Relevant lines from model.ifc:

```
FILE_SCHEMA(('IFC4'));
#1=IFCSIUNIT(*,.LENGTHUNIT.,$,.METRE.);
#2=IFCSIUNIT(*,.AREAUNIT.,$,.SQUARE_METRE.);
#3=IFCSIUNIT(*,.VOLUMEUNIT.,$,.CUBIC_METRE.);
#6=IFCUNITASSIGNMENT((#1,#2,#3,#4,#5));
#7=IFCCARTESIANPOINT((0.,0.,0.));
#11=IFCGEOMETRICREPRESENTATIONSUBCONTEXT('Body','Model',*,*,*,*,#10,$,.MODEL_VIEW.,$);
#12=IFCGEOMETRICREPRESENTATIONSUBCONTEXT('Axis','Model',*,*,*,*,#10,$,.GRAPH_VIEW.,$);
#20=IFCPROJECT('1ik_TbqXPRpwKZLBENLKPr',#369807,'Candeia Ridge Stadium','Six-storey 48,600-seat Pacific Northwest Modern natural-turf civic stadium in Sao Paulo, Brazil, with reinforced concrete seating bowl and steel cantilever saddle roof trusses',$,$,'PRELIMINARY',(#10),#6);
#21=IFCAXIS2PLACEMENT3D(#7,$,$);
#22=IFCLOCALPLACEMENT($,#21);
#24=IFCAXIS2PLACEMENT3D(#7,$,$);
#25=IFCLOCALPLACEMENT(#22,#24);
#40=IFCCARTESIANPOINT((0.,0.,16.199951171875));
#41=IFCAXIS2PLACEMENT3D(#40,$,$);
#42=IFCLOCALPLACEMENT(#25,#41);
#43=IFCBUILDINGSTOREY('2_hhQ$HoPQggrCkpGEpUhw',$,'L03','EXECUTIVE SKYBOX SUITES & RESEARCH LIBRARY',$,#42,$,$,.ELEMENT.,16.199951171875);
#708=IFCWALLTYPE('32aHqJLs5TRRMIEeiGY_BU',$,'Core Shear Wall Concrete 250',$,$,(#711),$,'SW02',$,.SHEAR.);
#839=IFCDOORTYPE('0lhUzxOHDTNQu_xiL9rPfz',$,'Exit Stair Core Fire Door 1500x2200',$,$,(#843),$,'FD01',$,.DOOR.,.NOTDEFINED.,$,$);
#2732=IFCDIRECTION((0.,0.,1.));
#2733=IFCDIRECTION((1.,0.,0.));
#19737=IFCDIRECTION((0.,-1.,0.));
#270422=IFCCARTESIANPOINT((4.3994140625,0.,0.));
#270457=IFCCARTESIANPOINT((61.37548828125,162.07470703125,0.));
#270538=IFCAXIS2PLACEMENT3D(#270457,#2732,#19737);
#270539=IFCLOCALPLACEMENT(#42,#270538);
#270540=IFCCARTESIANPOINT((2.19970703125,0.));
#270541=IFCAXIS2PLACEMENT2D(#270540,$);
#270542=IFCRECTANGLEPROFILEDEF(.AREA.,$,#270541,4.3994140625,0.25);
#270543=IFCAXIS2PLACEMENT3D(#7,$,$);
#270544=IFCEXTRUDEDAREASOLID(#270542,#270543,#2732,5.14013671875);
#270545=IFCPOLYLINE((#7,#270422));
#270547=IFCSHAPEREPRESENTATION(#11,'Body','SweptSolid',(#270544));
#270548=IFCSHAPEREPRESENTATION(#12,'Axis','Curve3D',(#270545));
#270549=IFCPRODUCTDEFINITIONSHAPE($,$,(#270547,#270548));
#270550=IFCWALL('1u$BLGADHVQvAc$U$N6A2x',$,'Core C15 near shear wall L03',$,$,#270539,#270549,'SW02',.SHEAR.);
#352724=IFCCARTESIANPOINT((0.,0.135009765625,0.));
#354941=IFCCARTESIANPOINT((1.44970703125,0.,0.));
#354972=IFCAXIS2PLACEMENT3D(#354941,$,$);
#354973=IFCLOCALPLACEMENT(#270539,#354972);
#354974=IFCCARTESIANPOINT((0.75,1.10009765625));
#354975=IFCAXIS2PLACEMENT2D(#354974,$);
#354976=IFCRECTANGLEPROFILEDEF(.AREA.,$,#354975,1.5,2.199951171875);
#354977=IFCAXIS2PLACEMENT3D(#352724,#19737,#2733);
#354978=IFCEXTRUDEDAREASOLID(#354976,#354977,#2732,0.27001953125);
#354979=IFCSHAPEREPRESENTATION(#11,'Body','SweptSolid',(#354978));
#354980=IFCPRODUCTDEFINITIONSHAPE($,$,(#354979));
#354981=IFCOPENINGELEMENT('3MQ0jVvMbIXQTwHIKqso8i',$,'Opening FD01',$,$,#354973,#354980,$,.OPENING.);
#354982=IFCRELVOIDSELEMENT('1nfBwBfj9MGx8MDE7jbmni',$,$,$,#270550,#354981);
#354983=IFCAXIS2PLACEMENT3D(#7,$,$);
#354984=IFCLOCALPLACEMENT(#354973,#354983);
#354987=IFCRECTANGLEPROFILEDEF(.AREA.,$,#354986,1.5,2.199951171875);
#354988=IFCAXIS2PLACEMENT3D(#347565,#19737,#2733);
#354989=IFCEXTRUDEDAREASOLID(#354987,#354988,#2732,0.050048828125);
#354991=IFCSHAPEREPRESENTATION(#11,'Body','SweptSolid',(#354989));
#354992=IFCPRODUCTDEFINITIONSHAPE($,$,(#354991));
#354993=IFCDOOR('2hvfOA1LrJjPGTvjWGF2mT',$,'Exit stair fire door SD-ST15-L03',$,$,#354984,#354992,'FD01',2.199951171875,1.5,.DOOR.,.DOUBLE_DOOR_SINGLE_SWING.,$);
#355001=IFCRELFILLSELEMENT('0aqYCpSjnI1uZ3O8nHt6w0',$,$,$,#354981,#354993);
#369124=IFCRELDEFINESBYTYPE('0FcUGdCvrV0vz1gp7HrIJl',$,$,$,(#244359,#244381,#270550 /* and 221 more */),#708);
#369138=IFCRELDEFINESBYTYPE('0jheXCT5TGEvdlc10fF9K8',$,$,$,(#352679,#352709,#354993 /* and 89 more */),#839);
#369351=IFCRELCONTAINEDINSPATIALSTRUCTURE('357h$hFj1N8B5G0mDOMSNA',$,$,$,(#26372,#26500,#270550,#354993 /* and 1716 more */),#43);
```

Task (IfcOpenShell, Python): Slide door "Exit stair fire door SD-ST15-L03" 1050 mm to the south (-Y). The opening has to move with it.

```python
import ifcopenshell
import ifcopenshell.api.geometry
import ifcopenshell.util.placement
import ifcopenshell.util.unit

model = ifcopenshell.open("model.ifc")
unit_scale = ifcopenshell.util.unit.calculate_unit_scale(model)

door = model.by_guid("2hvfOA1LrJjPGTvjWGF2mT")
opening = door.FillsVoids[0].RelatingOpeningElement
wall = opening.VoidsElements[0].RelatingBuildingElement

wall_matrix = ifcopenshell.util.placement.get_local_placement(wall.ObjectPlacement)
shift = wall_matrix[:3, 0] * 1.05 / unit_scale
before = ifcopenshell.util.placement.get_local_placement(door.ObjectPlacement)[:3, 3].copy()

# The door is placed relative to its opening, so it follows when the opening moves.
matrix = ifcopenshell.util.placement.get_local_placement(opening.ObjectPlacement)
matrix[:3, 3] += shift
ifcopenshell.api.geometry.edit_object_placement(
    model, product=opening, matrix=matrix, is_si=False, should_transform_children=True
)

after = ifcopenshell.util.placement.get_local_placement(door.ObjectPlacement)[:3, 3]
print("door moved by", (after - before).round(3) + 0.0)

model.write("model_edited.ifc")
```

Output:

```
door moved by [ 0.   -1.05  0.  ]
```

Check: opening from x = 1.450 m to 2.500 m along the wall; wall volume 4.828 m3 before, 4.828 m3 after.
